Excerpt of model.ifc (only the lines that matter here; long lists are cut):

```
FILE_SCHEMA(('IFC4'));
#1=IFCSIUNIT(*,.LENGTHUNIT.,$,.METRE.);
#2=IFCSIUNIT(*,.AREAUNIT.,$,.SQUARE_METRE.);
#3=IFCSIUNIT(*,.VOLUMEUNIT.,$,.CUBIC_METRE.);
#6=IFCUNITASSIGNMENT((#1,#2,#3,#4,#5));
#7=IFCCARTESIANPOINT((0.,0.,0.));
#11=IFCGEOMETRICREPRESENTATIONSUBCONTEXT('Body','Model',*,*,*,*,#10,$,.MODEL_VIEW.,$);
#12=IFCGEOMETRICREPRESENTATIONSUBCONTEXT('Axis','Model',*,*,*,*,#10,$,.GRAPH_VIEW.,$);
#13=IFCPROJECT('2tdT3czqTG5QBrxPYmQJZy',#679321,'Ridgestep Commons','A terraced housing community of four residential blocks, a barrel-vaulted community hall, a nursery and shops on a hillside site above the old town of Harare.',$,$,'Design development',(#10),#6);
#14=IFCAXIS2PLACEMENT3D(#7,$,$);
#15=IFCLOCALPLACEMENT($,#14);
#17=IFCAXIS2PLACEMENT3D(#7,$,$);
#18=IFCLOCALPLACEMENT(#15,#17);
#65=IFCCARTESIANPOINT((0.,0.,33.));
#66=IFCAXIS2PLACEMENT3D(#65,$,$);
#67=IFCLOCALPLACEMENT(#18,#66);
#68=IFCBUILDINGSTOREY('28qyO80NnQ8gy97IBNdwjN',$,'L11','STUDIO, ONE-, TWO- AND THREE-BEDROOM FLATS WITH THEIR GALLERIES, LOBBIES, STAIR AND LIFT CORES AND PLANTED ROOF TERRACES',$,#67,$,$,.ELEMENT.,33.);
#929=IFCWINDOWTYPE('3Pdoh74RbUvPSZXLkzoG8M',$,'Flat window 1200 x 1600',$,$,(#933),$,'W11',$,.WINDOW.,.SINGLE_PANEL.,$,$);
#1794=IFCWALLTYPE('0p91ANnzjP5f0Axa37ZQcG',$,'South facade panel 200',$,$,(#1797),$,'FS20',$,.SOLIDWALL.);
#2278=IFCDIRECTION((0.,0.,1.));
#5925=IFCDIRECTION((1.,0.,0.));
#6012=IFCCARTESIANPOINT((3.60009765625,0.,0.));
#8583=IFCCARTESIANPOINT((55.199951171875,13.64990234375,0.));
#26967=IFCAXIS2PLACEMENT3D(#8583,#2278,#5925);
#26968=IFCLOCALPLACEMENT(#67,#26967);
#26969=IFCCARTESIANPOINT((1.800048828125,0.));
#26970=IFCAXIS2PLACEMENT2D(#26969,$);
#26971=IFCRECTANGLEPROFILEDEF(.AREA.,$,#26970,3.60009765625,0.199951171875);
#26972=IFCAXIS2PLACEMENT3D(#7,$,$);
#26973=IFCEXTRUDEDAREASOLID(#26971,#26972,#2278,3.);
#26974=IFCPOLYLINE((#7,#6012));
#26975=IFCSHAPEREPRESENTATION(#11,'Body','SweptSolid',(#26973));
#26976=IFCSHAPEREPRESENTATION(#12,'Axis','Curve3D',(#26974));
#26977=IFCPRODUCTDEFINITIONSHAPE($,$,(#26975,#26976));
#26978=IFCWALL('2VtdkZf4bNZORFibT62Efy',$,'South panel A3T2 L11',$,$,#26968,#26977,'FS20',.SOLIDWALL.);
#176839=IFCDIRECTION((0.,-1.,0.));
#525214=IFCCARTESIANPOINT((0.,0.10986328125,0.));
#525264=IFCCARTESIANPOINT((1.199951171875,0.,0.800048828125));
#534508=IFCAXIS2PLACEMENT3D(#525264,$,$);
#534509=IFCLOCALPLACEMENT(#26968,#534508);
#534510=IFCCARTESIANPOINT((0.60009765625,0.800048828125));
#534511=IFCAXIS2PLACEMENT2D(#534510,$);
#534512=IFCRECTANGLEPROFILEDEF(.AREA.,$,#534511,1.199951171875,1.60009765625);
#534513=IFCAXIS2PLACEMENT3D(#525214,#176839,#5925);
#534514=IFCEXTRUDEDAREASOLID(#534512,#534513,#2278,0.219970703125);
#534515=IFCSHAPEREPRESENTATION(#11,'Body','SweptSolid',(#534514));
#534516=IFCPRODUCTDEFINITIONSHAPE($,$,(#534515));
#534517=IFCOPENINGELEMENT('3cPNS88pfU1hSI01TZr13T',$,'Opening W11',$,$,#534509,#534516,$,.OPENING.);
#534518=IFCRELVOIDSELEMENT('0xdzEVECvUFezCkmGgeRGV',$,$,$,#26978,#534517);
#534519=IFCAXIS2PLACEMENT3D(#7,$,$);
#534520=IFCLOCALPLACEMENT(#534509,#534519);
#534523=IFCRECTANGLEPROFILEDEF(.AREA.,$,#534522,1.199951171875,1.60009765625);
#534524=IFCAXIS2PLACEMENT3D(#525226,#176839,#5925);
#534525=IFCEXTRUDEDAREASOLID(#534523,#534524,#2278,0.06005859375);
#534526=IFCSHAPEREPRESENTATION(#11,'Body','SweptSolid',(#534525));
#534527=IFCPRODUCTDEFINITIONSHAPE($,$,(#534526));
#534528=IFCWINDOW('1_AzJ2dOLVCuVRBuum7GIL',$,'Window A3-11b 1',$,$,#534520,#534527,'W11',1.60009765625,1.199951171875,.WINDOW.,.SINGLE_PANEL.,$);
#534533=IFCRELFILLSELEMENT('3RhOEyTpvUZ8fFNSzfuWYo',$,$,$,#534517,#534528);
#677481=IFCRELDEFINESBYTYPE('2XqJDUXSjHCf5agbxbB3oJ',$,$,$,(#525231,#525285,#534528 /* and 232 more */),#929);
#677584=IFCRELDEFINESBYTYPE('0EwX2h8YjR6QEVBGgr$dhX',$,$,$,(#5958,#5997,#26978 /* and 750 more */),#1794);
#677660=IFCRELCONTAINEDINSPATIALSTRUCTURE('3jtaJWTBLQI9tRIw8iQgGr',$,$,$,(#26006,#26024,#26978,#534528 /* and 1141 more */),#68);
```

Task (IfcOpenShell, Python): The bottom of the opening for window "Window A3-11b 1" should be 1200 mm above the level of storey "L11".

```python
import numpy as np
import ifcopenshell
import ifcopenshell.api.geometry
import ifcopenshell.geom
import ifcopenshell.util.element
import ifcopenshell.util.placement
import ifcopenshell.util.shape
import ifcopenshell.util.unit

model = ifcopenshell.open("model.ifc")
unit_scale = ifcopenshell.util.unit.calculate_unit_scale(model)

window = model.by_guid("1_AzJ2dOLVCuVRBuum7GIL")
opening = window.FillsVoids[0].RelatingOpeningElement
storey = ifcopenshell.util.element.get_container(window, ifc_class="IfcBuildingStorey")
level = ifcopenshell.util.placement.get_local_placement(storey.ObjectPlacement)[2, 3]

# The opening's origin need not be at the sill, so measure its lowest point.
shape = ifcopenshell.geom.create_shape(ifcopenshell.geom.settings(), opening)
bottom = ifcopenshell.util.shape.get_shape_bottom_elevation(shape, shape.geometry) / unit_scale
dz = level + 1.2 / unit_scale - bottom

shift = np.array([0.0, 0.0, dz])
# The window is placed relative to its opening, so it follows when the opening moves.
matrix = ifcopenshell.util.placement.get_local_placement(opening.ObjectPlacement)
matrix[:3, 3] += shift
ifcopenshell.api.geometry.edit_object_placement(
    model, product=opening, matrix=matrix, is_si=False, should_transform_children=True
)

print(f"moved by {dz * unit_scale:+.3f} m")

model.write("model_edited.ifc")
```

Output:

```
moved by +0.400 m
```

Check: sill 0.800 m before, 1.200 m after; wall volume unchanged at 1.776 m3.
